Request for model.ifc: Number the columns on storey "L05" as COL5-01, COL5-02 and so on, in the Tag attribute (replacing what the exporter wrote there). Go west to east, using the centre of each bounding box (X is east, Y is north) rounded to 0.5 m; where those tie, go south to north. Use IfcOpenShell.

First a look at what the model holds.

```python
import ifcopenshell
import ifcopenshell.util.element
import ifcopenshell.util.placement

model = ifcopenshell.open("model.ifc")
print(model.schema)
storey = next(s for s in model.by_type("IfcBuildingStorey") if s.Name == "L05")
columns = [e for e in ifcopenshell.util.element.get_decomposition(storey) if e.is_a("IfcColumn")]
for e in sorted(columns, key=lambda e: e.id()):
    origin = ifcopenshell.util.placement.get_local_placement(e.ObjectPlacement)[:3, 3]
    print(e.id(), e.Tag, e.Name, origin.round(2) + 0.0, sep=" | ")
```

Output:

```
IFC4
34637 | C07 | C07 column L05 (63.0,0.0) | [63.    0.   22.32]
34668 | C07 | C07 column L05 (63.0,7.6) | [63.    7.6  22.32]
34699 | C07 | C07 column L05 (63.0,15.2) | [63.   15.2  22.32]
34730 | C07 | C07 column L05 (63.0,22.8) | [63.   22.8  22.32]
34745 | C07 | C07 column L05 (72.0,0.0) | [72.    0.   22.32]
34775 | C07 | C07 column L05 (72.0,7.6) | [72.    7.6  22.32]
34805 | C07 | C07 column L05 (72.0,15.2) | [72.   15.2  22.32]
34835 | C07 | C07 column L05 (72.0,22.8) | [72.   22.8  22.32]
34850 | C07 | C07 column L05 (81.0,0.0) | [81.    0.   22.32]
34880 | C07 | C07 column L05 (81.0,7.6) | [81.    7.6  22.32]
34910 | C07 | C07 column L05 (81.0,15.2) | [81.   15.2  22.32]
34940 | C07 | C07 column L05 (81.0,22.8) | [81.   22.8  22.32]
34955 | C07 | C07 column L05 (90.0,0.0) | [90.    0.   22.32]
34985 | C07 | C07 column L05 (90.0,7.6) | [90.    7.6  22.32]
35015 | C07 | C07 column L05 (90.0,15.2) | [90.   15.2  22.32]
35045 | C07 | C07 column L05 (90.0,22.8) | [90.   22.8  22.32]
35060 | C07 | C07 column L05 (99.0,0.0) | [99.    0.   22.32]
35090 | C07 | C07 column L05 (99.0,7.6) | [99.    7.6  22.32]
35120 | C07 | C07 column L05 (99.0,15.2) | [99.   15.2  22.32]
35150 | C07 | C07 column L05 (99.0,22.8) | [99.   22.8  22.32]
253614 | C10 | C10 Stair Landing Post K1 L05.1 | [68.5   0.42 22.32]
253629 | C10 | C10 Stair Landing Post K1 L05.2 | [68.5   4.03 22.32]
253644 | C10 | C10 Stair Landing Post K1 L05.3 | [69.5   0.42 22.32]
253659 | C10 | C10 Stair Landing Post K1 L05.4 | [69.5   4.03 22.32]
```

```python
import ifcopenshell
import ifcopenshell.geom
import ifcopenshell.util.element
import ifcopenshell.util.shape

model = ifcopenshell.open("model.ifc")
settings = ifcopenshell.geom.settings()
settings.set("use-world-coords", True)


def centre(element):
    shape = ifcopenshell.geom.create_shape(settings, element)
    return ifcopenshell.util.shape.get_bbox_centroid(shape.geometry)


storey = next(s for s in model.by_type("IfcBuildingStorey") if s.Name == "L05")
columns = [e for e in ifcopenshell.util.element.get_decomposition(storey) if e.is_a("IfcColumn")]

# Insertion points can sit at a corner or the storey origin, so sort by the geometry (in metres).
centres = {e: centre(e) for e in columns}
columns.sort(key=lambda e: (round(centres[e][0] / 0.5), centres[e][1]))

for i, e in enumerate(columns, start=1):
    number = f"COL5-{i:02d}"
    e.Tag = number
    print(e.id(), number)

model.write("model_updated.ifc")
```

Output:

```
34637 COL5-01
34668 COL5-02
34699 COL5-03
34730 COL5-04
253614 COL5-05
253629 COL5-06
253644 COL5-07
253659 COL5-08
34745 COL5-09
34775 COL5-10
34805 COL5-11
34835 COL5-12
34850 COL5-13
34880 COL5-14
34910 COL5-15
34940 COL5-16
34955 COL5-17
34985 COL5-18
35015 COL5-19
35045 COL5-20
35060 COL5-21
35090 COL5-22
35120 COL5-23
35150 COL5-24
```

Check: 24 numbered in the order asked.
